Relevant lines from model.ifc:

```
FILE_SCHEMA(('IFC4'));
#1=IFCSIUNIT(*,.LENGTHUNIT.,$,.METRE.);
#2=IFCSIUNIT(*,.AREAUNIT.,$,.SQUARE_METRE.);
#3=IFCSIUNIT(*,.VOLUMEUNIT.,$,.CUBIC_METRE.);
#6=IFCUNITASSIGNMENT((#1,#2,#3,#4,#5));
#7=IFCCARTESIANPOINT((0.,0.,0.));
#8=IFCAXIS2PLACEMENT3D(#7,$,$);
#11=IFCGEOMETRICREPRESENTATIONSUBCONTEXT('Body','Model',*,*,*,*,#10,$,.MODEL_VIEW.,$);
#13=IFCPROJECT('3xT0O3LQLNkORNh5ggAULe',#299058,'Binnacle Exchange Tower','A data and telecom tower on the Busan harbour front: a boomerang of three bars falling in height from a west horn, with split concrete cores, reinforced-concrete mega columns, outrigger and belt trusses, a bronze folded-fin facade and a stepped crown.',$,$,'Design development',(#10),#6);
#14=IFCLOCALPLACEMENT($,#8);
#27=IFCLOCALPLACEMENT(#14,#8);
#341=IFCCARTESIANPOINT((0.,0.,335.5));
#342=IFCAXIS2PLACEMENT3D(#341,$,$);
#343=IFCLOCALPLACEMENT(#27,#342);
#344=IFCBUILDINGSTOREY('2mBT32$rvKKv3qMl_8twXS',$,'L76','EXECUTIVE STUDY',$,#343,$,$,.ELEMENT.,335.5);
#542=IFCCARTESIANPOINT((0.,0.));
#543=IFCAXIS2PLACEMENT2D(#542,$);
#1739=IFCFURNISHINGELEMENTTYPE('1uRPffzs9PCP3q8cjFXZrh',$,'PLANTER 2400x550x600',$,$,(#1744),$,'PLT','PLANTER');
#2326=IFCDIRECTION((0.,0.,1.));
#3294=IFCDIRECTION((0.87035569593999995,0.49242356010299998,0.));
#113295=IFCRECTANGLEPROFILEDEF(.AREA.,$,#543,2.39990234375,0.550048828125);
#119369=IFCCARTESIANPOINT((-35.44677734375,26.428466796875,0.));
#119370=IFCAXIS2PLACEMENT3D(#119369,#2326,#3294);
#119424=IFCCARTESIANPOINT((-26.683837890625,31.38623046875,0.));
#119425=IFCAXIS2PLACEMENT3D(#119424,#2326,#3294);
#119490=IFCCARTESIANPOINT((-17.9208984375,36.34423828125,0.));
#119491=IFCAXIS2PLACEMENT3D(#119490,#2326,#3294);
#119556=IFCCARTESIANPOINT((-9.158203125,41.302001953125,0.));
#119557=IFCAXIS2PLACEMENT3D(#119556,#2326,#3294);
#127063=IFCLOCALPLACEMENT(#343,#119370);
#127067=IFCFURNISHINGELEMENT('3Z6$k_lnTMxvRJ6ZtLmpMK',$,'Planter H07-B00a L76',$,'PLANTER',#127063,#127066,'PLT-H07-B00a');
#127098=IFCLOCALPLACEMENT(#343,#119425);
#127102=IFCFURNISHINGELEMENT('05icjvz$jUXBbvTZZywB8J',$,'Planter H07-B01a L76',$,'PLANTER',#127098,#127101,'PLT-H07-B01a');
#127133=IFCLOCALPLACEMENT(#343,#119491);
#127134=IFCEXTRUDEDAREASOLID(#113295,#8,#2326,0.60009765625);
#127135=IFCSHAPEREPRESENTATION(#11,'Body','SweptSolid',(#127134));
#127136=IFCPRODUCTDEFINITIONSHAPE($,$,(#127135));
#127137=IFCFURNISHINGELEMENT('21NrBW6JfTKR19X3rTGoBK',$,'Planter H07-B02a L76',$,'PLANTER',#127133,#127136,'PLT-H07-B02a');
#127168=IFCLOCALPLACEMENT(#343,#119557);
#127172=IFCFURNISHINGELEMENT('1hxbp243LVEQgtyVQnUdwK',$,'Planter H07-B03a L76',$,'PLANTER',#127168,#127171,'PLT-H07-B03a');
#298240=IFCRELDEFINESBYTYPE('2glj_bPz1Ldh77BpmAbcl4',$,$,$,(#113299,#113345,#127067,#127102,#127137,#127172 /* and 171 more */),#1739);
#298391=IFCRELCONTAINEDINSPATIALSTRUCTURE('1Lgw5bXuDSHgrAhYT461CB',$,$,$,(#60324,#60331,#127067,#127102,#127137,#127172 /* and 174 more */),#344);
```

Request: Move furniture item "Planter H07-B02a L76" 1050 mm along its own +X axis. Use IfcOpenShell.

```python
import ifcopenshell
import ifcopenshell.api.geometry
import ifcopenshell.util.placement
import ifcopenshell.util.unit

model = ifcopenshell.open("model.ifc")
unit_scale = ifcopenshell.util.unit.calculate_unit_scale(model)

item = model.by_id(127137)
matrix = ifcopenshell.util.placement.get_local_placement(item.ObjectPlacement)
matrix[:3, 3] += matrix[:3, 0] * 1.05 / unit_scale
ifcopenshell.api.geometry.edit_object_placement(model, product=item, matrix=matrix, is_si=False)

print(ifcopenshell.util.placement.get_local_placement(item.ObjectPlacement).round(3) + 0.0)

model.write("model_edited.ifc")
```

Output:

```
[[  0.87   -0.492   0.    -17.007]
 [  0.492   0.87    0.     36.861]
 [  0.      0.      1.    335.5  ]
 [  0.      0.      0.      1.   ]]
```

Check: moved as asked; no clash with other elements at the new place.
